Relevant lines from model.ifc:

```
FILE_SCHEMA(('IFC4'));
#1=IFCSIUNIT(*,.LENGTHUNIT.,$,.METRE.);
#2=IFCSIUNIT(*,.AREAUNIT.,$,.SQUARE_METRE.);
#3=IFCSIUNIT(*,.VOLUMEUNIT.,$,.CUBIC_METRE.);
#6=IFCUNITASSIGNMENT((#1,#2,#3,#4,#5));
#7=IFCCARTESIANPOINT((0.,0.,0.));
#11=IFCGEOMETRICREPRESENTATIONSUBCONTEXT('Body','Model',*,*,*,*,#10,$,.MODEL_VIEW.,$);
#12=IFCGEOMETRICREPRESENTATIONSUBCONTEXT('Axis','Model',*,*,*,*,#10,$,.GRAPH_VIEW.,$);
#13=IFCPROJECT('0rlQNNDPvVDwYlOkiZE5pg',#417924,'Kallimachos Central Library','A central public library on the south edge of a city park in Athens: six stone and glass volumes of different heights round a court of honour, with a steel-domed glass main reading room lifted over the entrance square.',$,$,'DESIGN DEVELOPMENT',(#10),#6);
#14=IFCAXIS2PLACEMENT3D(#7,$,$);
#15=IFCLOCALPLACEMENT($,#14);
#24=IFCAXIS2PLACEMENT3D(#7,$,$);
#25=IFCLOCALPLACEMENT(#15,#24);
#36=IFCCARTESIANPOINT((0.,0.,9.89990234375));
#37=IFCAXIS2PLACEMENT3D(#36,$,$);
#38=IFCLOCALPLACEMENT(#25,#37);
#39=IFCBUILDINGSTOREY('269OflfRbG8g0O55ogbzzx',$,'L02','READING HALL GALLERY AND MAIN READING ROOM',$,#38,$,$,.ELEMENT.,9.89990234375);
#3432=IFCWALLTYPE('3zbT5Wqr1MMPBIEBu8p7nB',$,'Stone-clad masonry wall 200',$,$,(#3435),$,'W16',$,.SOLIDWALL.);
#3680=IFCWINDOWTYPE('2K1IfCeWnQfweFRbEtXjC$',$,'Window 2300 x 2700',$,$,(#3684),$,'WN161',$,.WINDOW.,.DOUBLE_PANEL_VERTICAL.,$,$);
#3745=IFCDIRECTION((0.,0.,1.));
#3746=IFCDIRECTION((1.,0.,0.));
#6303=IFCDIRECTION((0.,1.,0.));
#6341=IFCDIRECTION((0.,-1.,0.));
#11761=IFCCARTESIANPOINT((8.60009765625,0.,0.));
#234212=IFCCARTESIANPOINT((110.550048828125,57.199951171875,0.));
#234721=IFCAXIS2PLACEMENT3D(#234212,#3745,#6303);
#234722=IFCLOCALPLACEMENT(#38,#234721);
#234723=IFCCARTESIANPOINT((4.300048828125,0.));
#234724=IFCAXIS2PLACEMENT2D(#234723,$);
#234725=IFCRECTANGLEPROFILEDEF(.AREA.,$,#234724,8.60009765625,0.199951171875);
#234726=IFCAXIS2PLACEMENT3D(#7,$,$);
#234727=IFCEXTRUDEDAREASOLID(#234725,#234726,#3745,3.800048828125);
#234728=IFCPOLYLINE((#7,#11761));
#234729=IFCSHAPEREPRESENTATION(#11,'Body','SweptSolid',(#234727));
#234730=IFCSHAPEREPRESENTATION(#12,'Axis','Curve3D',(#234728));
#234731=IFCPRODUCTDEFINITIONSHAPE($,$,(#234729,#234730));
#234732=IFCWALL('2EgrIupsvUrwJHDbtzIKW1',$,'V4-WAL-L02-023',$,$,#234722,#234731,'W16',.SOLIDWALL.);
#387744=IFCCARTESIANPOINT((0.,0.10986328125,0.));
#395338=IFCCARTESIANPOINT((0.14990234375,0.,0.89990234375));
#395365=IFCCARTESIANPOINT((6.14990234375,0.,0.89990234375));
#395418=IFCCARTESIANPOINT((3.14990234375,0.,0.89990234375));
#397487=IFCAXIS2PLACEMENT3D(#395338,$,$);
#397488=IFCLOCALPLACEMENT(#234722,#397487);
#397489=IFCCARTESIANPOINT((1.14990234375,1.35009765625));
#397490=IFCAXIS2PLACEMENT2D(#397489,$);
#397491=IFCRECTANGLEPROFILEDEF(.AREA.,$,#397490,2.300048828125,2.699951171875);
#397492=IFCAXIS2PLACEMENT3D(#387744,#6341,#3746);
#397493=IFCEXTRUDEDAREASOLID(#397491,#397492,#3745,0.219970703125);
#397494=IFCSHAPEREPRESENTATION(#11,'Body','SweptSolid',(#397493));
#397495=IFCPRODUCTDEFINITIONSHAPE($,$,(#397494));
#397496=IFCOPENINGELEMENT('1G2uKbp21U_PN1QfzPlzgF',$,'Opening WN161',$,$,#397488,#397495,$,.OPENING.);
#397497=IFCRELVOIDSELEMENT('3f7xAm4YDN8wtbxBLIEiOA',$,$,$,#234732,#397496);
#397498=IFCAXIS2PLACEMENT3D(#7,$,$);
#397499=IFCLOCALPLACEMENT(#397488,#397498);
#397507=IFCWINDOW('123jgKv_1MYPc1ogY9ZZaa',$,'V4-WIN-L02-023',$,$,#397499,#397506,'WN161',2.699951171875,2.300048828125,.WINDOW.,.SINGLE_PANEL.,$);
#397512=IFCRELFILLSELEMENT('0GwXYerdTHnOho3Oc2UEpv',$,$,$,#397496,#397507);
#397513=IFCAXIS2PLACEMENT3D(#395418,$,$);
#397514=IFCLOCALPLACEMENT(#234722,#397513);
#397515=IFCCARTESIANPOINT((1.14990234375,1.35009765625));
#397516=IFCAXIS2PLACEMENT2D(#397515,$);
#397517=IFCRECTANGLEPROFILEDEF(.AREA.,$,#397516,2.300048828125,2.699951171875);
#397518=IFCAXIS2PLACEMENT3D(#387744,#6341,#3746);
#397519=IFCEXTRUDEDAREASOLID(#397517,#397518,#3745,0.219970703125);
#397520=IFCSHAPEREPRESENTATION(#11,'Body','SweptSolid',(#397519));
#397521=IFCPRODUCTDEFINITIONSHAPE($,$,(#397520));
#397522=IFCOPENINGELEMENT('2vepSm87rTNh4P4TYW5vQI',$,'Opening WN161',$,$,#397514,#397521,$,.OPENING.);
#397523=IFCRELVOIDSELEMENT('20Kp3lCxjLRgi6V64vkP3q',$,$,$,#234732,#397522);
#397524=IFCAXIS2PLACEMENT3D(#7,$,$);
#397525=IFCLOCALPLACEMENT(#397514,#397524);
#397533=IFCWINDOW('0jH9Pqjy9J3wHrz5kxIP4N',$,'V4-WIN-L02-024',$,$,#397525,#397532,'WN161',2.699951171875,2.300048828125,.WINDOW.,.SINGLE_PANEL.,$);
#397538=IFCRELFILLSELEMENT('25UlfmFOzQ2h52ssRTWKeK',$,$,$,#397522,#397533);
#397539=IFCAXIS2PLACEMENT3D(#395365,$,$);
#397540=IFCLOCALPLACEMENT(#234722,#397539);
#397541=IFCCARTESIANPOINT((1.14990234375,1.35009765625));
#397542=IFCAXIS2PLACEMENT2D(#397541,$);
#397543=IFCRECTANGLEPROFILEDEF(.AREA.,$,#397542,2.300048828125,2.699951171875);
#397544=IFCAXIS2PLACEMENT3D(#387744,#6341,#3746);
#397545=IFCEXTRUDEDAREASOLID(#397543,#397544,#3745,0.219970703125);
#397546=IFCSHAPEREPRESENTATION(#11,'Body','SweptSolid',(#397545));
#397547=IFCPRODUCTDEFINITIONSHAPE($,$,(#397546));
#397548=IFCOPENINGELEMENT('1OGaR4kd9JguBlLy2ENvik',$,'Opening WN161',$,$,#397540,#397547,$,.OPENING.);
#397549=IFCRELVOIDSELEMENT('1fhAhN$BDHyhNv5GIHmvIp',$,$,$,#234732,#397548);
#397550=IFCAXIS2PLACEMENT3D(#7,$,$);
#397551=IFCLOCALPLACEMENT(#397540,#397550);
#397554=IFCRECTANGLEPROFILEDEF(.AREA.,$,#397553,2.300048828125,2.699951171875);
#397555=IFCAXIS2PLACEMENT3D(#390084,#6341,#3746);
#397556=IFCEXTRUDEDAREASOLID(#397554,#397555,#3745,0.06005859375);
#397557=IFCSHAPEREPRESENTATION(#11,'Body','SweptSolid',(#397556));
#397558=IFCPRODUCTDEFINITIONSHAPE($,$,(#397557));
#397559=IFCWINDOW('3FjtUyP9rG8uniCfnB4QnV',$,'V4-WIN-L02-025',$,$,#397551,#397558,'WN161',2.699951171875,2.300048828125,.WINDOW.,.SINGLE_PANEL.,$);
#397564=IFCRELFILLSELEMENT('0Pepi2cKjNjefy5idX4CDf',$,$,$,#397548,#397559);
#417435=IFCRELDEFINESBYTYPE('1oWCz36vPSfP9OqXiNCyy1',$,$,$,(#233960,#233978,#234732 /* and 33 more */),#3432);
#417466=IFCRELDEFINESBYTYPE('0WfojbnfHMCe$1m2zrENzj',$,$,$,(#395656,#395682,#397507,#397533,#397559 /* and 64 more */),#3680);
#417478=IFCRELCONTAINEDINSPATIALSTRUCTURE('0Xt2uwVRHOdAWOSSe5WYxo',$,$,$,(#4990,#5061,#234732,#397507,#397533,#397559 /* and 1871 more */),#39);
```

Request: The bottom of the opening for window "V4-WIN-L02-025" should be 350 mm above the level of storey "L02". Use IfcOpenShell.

```python
import numpy as np
import ifcopenshell
import ifcopenshell.api.geometry
import ifcopenshell.geom
import ifcopenshell.util.element
import ifcopenshell.util.placement
import ifcopenshell.util.shape
import ifcopenshell.util.unit

model = ifcopenshell.open("model.ifc")
unit_scale = ifcopenshell.util.unit.calculate_unit_scale(model)

window = model.by_guid("3FjtUyP9rG8uniCfnB4QnV")
opening = window.FillsVoids[0].RelatingOpeningElement
storey = ifcopenshell.util.element.get_container(window, ifc_class="IfcBuildingStorey")
level = ifcopenshell.util.placement.get_local_placement(storey.ObjectPlacement)[2, 3]

# The opening's origin need not be at the sill, so measure its lowest point.
shape = ifcopenshell.geom.create_shape(ifcopenshell.geom.settings(), opening)
bottom = ifcopenshell.util.shape.get_shape_bottom_elevation(shape, shape.geometry) / unit_scale
dz = level + 0.35 - bottom

shift = np.array([0.0, 0.0, dz])
# The window is placed relative to its opening, so it follows when the opening moves.
matrix = ifcopenshell.util.placement.get_local_placement(opening.ObjectPlacement)
matrix[:3, 3] += shift
ifcopenshell.api.geometry.edit_object_placement(
    model, product=opening, matrix=matrix, is_si=False, should_transform_children=True
)

print(f"moved by {dz * unit_scale:+.3f} m")

model.write("model-out.ifc")
```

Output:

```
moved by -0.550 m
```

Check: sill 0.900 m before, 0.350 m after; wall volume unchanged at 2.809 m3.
